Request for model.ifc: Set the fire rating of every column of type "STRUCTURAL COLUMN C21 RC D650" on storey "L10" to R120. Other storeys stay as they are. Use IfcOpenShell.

First a look at what the model holds.

```python
import ifcopenshell
import ifcopenshell.util.element

model = ifcopenshell.open("model.ifc")
print(model.schema)
storey = next(s for s in model.by_type("IfcBuildingStorey") if s.Name == "L10")
columns = [e for e in ifcopenshell.util.element.get_decomposition(storey) if e.is_a("IfcColumn")]
seen = {}
for e in columns:
    element_type = ifcopenshell.util.element.get_type(e)
    key = (element_type.Name if element_type != e and element_type else None, ifcopenshell.util.element.get_pset(e, "Pset_ColumnCommon", "FireRating"))
    seen[key] = seen.get(key, 0) + 1
for (name, value), count in sorted(seen.items(), key=str):
    print(count, "x", name, "|", value)
```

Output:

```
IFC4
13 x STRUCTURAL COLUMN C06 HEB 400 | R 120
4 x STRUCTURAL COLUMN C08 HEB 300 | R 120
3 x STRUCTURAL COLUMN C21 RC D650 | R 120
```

```python
import ifcopenshell
import ifcopenshell.api.pset
import ifcopenshell.util.element

model = ifcopenshell.open("model.ifc")

storey = next(s for s in model.by_type("IfcBuildingStorey") if s.Name == "L10")
columns = [e for e in ifcopenshell.util.element.get_decomposition(storey) if e.is_a("IfcColumn")]

count = 0
for e in columns:
    element_type = ifcopenshell.util.element.get_type(e)
    if element_type in (None, e) or element_type.Name != "STRUCTURAL COLUMN C21 RC D650":
        continue
    # add_pset returns the element's existing set when there is one.
    pset = ifcopenshell.api.pset.add_pset(model, product=e, name="Pset_ColumnCommon")
    ifcopenshell.api.pset.edit_pset(model, pset=pset, properties={"FireRating": "R120"})
    count += 1

print(count, "columns updated")

model.write("model_updated.ifc")
```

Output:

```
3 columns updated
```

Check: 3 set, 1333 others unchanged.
